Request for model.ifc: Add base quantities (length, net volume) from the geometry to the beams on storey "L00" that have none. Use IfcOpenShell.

First a look at what the model holds.

```python
import ifcopenshell
import ifcopenshell.util.element
import ifcopenshell.util.unit

model = ifcopenshell.open("model.ifc")
print(model.schema)
for unit_type in ("LENGTHUNIT", "AREAUNIT", "VOLUMEUNIT"):
    print(unit_type, ifcopenshell.util.unit.calculate_unit_scale(model, unit_type))
storey = next(s for s in model.by_type("IfcBuildingStorey") if s.Name == "L00")
beams = [e for e in ifcopenshell.util.element.get_decomposition(storey) if e.is_a("IfcBeam")]
for e in sorted(beams, key=lambda e: e.id()):
    print(e.id(), e.is_a(), e.Name, list(ifcopenshell.util.element.get_psets(e, qtos_only=True)), sep=" | ")
```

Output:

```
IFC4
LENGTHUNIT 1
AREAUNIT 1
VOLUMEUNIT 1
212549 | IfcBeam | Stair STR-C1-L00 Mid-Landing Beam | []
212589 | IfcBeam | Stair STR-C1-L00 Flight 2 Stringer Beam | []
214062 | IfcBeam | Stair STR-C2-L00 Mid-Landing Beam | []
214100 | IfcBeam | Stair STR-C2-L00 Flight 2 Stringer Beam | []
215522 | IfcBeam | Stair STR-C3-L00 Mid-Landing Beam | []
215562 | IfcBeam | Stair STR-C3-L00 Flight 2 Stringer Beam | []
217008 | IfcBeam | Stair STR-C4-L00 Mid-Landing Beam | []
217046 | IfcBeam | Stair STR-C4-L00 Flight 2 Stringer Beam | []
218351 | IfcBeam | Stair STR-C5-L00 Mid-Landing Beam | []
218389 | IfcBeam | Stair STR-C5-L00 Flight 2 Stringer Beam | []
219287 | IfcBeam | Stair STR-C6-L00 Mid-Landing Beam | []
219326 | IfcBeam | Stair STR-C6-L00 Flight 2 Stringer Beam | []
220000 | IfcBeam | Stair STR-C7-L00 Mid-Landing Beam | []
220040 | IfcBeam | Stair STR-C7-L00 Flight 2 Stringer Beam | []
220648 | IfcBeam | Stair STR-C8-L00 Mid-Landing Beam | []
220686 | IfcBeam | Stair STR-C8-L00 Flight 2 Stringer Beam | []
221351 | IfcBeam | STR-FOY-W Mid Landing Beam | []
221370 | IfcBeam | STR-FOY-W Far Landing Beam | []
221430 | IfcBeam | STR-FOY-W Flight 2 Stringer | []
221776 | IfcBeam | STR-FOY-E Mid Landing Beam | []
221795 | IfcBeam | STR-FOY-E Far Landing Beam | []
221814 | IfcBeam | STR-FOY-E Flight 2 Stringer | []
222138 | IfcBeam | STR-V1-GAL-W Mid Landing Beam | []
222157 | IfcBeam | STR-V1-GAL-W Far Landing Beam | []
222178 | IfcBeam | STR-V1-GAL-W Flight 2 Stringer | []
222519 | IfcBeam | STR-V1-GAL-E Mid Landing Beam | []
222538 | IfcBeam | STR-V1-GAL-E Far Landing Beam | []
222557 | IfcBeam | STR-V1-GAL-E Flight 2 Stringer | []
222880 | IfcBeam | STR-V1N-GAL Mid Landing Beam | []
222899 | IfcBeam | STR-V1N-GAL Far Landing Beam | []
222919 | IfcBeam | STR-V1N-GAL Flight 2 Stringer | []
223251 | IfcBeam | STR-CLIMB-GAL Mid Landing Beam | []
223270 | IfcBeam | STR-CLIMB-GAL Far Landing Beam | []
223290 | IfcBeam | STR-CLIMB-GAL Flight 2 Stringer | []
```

```python
import ifcopenshell
import ifcopenshell.api.pset
import ifcopenshell.geom
import ifcopenshell.util.element
import ifcopenshell.util.shape
import ifcopenshell.util.unit

model = ifcopenshell.open("model.ifc")
unit_scale = ifcopenshell.util.unit.calculate_unit_scale(model)
volume_scale = ifcopenshell.util.unit.calculate_unit_scale(model, "VOLUMEUNIT")
settings = ifcopenshell.geom.settings()

storey = next(s for s in model.by_type("IfcBuildingStorey") if s.Name == "L00")
beams = [e for e in ifcopenshell.util.element.get_decomposition(storey) if e.is_a("IfcBeam")]

for e in sorted(beams, key=lambda e: e.id()):
    if ifcopenshell.util.element.get_psets(e, qtos_only=True, should_inherit=False):
        continue
    # Geometry comes back in metres, in the element's own axes.
    shape = ifcopenshell.geom.create_shape(settings, e)
    values = {
        "Length": ifcopenshell.util.shape.get_max_xyz(shape.geometry) / unit_scale,
        "NetVolume": ifcopenshell.util.shape.get_volume(shape.geometry) / volume_scale,
    }
    qto = ifcopenshell.api.pset.add_qto(model, product=e, name="Qto_BeamBaseQuantities")
    ifcopenshell.api.pset.edit_qto(model, qto=qto, properties=values)
    print(e.id(), {k: round(v, 3) for k, v in values.items()})

model.write("model_v2.ifc")
```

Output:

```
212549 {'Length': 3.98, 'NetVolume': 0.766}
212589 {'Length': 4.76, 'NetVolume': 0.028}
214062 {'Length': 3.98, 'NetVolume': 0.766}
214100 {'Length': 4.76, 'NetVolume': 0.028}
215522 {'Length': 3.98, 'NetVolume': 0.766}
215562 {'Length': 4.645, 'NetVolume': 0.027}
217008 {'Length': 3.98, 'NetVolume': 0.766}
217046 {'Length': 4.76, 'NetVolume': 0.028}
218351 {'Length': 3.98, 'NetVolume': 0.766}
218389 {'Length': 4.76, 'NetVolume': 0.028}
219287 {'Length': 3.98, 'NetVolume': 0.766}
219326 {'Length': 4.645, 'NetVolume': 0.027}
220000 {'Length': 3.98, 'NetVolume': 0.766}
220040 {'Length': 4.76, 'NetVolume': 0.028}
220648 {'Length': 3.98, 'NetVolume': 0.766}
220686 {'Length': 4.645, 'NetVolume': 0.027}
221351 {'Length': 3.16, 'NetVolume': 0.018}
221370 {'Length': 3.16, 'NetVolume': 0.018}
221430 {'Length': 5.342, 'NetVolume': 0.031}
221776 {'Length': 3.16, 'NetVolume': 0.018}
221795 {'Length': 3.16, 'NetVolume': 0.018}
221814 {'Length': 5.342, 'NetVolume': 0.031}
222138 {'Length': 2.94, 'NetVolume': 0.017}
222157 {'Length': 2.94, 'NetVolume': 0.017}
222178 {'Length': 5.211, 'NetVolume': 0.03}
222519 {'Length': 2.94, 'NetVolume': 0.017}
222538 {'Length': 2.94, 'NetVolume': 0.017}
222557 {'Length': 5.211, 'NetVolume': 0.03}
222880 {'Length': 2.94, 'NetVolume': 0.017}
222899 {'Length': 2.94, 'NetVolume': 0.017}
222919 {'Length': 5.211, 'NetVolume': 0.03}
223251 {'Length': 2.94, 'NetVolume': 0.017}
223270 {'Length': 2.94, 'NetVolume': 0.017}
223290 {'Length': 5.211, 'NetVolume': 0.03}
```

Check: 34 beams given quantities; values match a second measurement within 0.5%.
